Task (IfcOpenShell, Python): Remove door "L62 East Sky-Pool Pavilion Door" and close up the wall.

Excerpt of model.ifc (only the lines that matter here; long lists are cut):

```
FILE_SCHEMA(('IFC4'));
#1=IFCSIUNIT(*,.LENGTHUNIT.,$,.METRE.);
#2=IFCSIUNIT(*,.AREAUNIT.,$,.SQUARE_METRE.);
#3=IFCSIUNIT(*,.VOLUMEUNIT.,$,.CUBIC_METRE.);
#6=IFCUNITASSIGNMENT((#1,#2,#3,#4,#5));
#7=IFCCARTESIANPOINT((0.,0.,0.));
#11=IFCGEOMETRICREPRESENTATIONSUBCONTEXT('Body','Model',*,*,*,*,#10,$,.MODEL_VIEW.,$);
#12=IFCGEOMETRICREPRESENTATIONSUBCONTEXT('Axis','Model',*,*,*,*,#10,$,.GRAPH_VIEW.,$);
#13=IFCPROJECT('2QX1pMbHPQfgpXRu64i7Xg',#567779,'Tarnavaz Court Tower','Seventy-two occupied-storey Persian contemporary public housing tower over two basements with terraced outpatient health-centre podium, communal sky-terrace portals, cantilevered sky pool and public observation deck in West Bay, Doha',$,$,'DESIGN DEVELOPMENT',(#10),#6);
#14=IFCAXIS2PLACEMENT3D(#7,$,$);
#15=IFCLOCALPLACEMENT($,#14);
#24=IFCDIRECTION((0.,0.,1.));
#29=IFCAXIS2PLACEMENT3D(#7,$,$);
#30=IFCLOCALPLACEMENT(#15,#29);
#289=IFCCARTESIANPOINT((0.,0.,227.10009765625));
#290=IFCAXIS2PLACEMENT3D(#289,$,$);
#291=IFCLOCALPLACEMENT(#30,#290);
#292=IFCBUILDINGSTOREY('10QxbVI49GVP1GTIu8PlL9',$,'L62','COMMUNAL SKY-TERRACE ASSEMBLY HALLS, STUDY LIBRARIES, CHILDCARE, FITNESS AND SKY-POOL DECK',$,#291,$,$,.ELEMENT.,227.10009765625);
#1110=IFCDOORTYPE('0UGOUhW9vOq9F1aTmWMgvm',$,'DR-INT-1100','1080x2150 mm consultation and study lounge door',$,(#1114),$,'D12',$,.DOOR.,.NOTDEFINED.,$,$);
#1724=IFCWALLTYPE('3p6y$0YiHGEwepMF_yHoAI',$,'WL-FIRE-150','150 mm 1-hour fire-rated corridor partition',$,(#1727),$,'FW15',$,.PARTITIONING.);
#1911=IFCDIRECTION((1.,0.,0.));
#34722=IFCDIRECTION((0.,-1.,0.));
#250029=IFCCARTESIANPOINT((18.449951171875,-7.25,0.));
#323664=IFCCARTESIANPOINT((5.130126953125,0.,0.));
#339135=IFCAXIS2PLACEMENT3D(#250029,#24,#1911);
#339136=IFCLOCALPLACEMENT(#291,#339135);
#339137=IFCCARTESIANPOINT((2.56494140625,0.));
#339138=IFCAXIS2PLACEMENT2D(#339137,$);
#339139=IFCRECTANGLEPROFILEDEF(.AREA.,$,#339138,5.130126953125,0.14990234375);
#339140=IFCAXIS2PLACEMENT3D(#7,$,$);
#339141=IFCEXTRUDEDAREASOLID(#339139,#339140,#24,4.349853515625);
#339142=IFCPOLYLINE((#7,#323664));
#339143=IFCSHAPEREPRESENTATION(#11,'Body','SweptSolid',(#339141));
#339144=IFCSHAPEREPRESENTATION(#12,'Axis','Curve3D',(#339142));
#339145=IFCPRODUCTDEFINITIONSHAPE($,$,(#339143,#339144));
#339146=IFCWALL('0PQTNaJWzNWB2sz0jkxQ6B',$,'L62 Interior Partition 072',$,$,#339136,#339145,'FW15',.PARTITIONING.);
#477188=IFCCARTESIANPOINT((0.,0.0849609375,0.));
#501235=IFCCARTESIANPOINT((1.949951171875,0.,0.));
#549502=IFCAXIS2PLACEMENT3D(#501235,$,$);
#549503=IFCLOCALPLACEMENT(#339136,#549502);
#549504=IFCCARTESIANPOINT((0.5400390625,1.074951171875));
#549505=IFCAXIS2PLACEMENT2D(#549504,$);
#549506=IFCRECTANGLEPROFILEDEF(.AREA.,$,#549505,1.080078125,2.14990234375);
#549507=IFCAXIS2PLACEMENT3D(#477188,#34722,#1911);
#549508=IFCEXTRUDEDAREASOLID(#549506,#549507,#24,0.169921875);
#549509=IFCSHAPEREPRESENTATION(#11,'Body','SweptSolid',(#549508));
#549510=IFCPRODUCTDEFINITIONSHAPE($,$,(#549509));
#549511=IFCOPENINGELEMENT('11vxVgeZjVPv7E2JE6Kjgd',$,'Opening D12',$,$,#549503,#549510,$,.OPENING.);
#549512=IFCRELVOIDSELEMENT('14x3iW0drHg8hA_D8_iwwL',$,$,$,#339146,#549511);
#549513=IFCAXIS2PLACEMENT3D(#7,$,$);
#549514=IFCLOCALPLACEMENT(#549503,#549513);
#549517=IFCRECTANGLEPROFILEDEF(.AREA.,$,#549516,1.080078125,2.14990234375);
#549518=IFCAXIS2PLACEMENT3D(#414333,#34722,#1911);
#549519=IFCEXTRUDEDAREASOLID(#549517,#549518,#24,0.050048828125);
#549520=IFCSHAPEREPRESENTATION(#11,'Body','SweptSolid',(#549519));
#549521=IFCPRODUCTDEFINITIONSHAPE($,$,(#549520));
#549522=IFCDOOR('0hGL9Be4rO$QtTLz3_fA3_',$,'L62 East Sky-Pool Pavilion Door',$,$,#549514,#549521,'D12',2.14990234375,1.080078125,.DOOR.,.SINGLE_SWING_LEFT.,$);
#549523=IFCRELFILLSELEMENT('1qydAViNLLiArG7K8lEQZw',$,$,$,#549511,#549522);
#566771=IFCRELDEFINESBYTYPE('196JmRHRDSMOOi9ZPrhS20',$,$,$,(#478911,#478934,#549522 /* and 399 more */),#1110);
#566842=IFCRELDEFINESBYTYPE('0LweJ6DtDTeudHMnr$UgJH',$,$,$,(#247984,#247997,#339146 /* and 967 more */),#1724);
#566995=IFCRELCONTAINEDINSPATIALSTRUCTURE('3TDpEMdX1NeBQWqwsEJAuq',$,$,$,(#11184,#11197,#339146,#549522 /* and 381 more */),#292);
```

```python
import ifcopenshell
import ifcopenshell.api.feature
import ifcopenshell.api.root
import ifcopenshell.geom
import ifcopenshell.util.shape

model = ifcopenshell.open("model.ifc")
settings = ifcopenshell.geom.settings()


def volume(element):
    """Net volume in cubic metres, openings subtracted."""
    shape = ifcopenshell.geom.create_shape(settings, element)
    return ifcopenshell.util.shape.get_volume(shape.geometry)


door = model.by_id(549522)
opening = door.FillsVoids[0].RelatingOpeningElement
wall = opening.VoidsElements[0].RelatingBuildingElement
before = volume(wall)

ifcopenshell.api.root.remove_product(model, product=door)
ifcopenshell.api.feature.remove_feature(model, feature=opening)

after = volume(wall)

print(f"wall volume {before:.3f} -> {after:.3f} m3")

model.write("model_v2.ifc")
```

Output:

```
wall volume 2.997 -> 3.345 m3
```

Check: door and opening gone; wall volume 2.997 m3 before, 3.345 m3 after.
